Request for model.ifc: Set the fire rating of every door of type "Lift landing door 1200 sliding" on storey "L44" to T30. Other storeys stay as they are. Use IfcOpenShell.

First a look at what the model holds.

```python
import ifcopenshell
import ifcopenshell.util.element

model = ifcopenshell.open("model.ifc")
print(model.schema)
storey = next(s for s in model.by_type("IfcBuildingStorey") if s.Name == "L44")
doors = [e for e in ifcopenshell.util.element.get_decomposition(storey) if e.is_a("IfcDoor")]
seen = {}
for e in doors:
    element_type = ifcopenshell.util.element.get_type(e)
    key = (element_type.Name if element_type != e and element_type else None, ifcopenshell.util.element.get_pset(e, "Pset_DoorCommon", "FireRating"))
    seen[key] = seen.get(key, 0) + 1
for (name, value), count in sorted(seen.items(), key=str):
    print(count, "x", name, "|", value)
```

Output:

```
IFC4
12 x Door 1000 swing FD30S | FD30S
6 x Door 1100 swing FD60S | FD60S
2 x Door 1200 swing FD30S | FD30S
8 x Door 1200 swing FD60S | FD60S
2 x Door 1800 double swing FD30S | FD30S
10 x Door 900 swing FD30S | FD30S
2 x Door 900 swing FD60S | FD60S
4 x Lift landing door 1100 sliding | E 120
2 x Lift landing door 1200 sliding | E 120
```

```python
import ifcopenshell
import ifcopenshell.api.pset
import ifcopenshell.util.element

model = ifcopenshell.open("model.ifc")

storey = next(s for s in model.by_type("IfcBuildingStorey") if s.Name == "L44")
doors = [e for e in ifcopenshell.util.element.get_decomposition(storey) if e.is_a("IfcDoor")]

count = 0
for e in doors:
    element_type = ifcopenshell.util.element.get_type(e)
    if element_type in (None, e) or element_type.Name != "Lift landing door 1200 sliding":
        continue
    # add_pset returns the element's existing set when there is one.
    pset = ifcopenshell.api.pset.add_pset(model, product=e, name="Pset_DoorCommon")
    ifcopenshell.api.pset.edit_pset(model, pset=pset, properties={"FireRating": "T30"})
    count += 1

print(count, "doors updated")

model.write("model_updated.ifc")
```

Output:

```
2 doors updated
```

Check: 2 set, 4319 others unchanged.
